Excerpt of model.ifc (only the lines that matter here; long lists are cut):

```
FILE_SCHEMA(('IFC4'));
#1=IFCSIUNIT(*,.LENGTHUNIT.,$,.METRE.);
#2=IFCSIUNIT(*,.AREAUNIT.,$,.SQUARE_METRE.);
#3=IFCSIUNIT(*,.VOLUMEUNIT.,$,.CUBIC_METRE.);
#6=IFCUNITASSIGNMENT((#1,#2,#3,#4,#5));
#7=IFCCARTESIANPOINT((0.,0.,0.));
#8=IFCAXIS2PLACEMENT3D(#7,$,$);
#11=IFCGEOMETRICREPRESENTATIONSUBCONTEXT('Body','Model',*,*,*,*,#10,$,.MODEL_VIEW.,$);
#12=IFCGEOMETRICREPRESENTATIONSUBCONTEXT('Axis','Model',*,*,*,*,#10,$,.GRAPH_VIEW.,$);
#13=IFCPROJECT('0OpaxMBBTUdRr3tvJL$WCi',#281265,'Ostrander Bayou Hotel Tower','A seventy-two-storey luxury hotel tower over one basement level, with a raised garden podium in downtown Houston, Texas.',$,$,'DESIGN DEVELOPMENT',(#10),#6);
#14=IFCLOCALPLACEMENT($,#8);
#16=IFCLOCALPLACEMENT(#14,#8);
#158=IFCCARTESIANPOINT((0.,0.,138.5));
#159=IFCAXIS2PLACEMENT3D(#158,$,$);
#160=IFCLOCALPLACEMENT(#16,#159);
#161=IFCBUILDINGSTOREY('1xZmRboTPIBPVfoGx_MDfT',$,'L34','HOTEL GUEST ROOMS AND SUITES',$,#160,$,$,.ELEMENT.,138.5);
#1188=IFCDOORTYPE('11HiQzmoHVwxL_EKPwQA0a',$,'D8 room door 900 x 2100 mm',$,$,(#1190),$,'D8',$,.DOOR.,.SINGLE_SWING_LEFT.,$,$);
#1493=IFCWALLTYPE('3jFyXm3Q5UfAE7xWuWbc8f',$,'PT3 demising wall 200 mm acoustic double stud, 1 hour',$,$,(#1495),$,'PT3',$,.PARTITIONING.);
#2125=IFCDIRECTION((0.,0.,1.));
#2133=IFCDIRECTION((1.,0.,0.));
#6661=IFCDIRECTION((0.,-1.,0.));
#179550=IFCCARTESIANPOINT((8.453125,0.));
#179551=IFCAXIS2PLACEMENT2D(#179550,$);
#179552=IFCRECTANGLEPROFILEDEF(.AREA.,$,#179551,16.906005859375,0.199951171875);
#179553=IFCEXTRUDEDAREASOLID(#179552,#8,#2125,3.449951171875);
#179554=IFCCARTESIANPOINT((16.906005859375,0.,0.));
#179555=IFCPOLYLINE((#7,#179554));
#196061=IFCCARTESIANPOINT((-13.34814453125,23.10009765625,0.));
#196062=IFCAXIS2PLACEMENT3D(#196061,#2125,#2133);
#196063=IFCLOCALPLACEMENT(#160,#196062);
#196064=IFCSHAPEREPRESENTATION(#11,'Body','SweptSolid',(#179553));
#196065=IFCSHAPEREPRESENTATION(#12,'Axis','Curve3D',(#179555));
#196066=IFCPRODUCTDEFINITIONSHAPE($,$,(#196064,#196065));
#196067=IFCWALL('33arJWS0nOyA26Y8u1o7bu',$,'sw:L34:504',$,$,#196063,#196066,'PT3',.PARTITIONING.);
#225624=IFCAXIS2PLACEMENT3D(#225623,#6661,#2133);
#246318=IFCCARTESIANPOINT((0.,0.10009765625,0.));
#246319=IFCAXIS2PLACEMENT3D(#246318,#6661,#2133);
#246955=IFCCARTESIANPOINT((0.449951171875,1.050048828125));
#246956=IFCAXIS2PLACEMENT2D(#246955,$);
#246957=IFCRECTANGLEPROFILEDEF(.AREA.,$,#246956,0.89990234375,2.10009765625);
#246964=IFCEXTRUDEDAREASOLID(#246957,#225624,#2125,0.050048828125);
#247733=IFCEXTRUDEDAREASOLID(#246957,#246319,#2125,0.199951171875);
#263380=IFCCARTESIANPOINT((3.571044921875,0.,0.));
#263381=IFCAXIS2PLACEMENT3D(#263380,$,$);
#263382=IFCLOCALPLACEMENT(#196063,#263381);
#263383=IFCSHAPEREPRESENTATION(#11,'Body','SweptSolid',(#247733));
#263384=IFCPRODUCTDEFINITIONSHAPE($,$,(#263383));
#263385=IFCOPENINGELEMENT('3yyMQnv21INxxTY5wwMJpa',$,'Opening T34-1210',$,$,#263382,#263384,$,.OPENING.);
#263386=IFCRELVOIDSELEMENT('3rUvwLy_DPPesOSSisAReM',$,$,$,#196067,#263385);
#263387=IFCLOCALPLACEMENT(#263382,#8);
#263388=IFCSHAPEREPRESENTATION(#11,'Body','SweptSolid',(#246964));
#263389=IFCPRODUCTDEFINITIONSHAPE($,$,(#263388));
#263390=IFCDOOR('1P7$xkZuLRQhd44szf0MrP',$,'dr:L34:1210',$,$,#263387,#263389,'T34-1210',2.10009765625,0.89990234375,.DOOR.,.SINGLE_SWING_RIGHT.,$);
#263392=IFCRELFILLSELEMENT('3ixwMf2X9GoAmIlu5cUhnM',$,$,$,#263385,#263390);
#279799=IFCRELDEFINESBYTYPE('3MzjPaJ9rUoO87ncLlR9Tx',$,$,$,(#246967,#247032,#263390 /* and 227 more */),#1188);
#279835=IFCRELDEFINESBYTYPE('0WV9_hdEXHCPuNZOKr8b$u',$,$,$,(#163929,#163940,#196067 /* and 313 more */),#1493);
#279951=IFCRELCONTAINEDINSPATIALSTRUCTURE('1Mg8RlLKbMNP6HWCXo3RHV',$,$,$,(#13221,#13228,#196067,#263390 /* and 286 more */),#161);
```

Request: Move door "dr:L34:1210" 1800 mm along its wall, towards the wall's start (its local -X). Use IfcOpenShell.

```python
import ifcopenshell
import ifcopenshell.api.geometry
import ifcopenshell.util.placement

model = ifcopenshell.open("model.ifc")

door = model.by_guid("1P7$xkZuLRQhd44szf0MrP")
opening = door.FillsVoids[0].RelatingOpeningElement
wall = opening.VoidsElements[0].RelatingBuildingElement

wall_matrix = ifcopenshell.util.placement.get_local_placement(wall.ObjectPlacement)
shift = wall_matrix[:3, 0] * -1.8
before = ifcopenshell.util.placement.get_local_placement(door.ObjectPlacement)[:3, 3].copy()

# The door is placed relative to its opening, so it follows when the opening moves.
matrix = ifcopenshell.util.placement.get_local_placement(opening.ObjectPlacement)
matrix[:3, 3] += shift
ifcopenshell.api.geometry.edit_object_placement(
    model, product=opening, matrix=matrix, is_si=False, should_transform_children=True
)

after = ifcopenshell.util.placement.get_local_placement(door.ObjectPlacement)[:3, 3]
print("door moved by", (after - before).round(3) + 0.0)

model.write("model_updated.ifc")
```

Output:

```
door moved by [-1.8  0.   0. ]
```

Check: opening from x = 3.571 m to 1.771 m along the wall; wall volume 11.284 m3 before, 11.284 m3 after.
